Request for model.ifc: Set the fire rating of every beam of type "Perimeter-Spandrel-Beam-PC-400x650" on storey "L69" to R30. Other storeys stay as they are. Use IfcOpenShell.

First a look at what the model holds.

```python
import ifcopenshell
import ifcopenshell.util.element

model = ifcopenshell.open("model.ifc")
print(model.schema)
storey = next(s for s in model.by_type("IfcBuildingStorey") if s.Name == "L69")
beams = [e for e in ifcopenshell.util.element.get_decomposition(storey) if e.is_a("IfcBeam")]
seen = {}
for e in beams:
    element_type = ifcopenshell.util.element.get_type(e)
    key = (element_type.Name if element_type != e and element_type else None, ifcopenshell.util.element.get_pset(e, "Pset_BeamCommon", "FireRating"))
    seen[key] = seen.get(key, 0) + 1
for (name, value), count in sorted(seen.items(), key=str):
    print(count, "x", name, "|", value)
```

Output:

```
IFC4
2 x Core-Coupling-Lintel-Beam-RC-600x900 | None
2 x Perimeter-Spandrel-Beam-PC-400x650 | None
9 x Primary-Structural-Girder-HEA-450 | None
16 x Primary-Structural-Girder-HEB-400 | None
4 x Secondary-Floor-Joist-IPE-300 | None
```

```python
import ifcopenshell
import ifcopenshell.api.pset
import ifcopenshell.util.element

model = ifcopenshell.open("model.ifc")

storey = next(s for s in model.by_type("IfcBuildingStorey") if s.Name == "L69")
beams = [e for e in ifcopenshell.util.element.get_decomposition(storey) if e.is_a("IfcBeam")]

count = 0
for e in beams:
    element_type = ifcopenshell.util.element.get_type(e)
    if element_type in (None, e) or element_type.Name != "Perimeter-Spandrel-Beam-PC-400x650":
        continue
    found = ifcopenshell.util.element.get_pset(e, "Pset_BeamCommon", should_inherit=False)
    if found:
        pset = model.by_id(found["id"])
        if len(ifcopenshell.util.element.get_elements_by_pset(pset)) > 1:
            pset = ifcopenshell.api.pset.unshare_pset(model, products=[e], pset=pset)[0]
    else:
        pset = ifcopenshell.api.pset.add_pset(model, product=e, name="Pset_BeamCommon")
    ifcopenshell.api.pset.edit_pset(model, pset=pset, properties={"FireRating": "R30"})
    count += 1

print(count, "beams updated")

model.write("model-out.ifc")
```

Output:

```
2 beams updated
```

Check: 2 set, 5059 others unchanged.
